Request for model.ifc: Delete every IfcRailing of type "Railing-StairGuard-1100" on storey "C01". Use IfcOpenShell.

First a look at what the model holds.

```python
import ifcopenshell
import ifcopenshell.util.element

model = ifcopenshell.open("model.ifc")
print(model.schema)
storey = next(s for s in model.by_type("IfcBuildingStorey") if s.Name == "C01")
railings = [e for e in ifcopenshell.util.element.get_decomposition(storey) if e.is_a("IfcRailing")]
seen = {}
for e in railings:
    element_type = ifcopenshell.util.element.get_type(e)
    name = element_type.Name if element_type not in (None, e) else None
    seen[name] = seen.get(name, 0) + 1
for name, count in sorted(seen.items(), key=str):
    print(count, "x", name)
```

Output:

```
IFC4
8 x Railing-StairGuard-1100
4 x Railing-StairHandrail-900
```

```python
import ifcopenshell
import ifcopenshell.api.root
import ifcopenshell.util.element

model = ifcopenshell.open("model.ifc")

storey = next(s for s in model.by_type("IfcBuildingStorey") if s.Name == "C01")
railings = [e for e in ifcopenshell.util.element.get_decomposition(storey) if e.is_a("IfcRailing")]
targets = [e for e in railings if (t := ifcopenshell.util.element.get_type(e)) not in (None, e) and t.Name == "Railing-StairGuard-1100"]

for e in targets:
    ifcopenshell.api.root.remove_product(model, product=e)
print(len(targets), "removed")

model.write("model_updated.ifc")
```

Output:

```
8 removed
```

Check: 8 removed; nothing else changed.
